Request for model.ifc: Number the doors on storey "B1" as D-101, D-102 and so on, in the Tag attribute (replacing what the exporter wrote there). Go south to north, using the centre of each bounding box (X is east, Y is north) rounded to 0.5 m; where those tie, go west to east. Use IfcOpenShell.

First a look at what the model holds.

```python
import ifcopenshell
import ifcopenshell.util.element
import ifcopenshell.util.placement

model = ifcopenshell.open("model.ifc")
print(model.schema)
storey = next(s for s in model.by_type("IfcBuildingStorey") if s.Name == "B1")
doors = [e for e in ifcopenshell.util.element.get_decomposition(storey) if e.is_a("IfcDoor")]
for e in sorted(doors, key=lambda e: e.id()):
    origin = ifcopenshell.util.placement.get_local_placement(e.ObjectPlacement)[:3, 3]
    print(e.id(), e.Tag, e.Name, origin.round(2) + 0.0, sep=" | ")
```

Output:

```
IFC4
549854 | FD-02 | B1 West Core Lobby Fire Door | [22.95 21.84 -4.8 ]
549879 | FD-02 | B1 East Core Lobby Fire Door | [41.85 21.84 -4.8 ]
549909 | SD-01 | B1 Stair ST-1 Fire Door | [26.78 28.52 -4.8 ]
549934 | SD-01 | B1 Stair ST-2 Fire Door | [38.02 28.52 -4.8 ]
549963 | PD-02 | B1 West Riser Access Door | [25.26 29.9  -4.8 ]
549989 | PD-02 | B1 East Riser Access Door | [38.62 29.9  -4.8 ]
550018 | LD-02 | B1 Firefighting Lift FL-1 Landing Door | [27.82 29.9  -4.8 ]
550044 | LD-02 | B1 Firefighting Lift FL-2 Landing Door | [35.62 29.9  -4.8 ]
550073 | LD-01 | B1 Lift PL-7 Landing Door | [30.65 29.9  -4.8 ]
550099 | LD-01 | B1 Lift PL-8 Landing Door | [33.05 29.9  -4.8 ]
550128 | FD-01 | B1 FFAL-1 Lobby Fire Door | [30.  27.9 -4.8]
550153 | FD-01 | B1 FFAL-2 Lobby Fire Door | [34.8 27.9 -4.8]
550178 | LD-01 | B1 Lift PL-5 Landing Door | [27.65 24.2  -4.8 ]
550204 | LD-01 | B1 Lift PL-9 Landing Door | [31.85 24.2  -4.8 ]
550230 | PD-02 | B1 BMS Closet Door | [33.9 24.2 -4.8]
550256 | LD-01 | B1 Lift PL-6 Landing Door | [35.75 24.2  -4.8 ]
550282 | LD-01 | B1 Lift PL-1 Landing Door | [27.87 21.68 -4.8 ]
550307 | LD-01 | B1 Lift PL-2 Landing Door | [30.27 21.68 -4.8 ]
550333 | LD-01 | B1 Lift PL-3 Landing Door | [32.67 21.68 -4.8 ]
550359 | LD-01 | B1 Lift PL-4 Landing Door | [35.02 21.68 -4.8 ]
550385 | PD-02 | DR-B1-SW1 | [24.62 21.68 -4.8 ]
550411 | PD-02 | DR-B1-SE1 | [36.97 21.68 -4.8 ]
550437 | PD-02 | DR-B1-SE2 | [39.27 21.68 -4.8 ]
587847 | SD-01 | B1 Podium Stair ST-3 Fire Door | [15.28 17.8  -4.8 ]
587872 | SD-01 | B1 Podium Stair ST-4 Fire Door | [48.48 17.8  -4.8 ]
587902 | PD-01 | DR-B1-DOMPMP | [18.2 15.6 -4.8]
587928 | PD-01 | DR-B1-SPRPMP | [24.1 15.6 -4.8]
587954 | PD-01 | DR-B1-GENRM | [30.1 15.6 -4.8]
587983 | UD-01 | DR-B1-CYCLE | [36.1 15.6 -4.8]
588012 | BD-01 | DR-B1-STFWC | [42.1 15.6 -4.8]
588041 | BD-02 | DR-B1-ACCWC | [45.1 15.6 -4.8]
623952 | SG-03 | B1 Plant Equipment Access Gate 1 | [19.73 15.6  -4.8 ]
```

```python
import ifcopenshell
import ifcopenshell.geom
import ifcopenshell.util.element
import ifcopenshell.util.shape

model = ifcopenshell.open("model.ifc")
settings = ifcopenshell.geom.settings()
settings.set("use-world-coords", True)


def centre(element):
    shape = ifcopenshell.geom.create_shape(settings, element)
    return ifcopenshell.util.shape.get_bbox_centroid(shape.geometry)


storey = next(s for s in model.by_type("IfcBuildingStorey") if s.Name == "B1")
doors = [e for e in ifcopenshell.util.element.get_decomposition(storey) if e.is_a("IfcDoor")]

# Insertion points can sit at a corner or the storey origin, so sort by the geometry (in metres).
centres = {e: centre(e) for e in doors}
doors.sort(key=lambda e: (round(centres[e][1] / 0.5), centres[e][0]))

for i, e in enumerate(doors, start=1):
    number = f"D-1{i:02d}"
    e.Tag = number
    print(e.id(), number)

model.write("model-out.ifc")
```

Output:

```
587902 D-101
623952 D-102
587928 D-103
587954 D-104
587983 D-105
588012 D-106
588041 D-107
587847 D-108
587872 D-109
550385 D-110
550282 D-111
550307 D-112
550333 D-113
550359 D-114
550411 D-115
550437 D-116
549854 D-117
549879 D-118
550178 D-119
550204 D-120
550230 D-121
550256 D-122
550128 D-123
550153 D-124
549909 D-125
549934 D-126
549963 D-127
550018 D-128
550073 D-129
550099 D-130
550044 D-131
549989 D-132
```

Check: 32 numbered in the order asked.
